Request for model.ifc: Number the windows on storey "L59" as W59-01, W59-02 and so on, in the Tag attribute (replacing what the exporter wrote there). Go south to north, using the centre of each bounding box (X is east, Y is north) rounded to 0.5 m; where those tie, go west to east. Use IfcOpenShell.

First a look at what the model holds.

```python
import ifcopenshell
import ifcopenshell.util.element
import ifcopenshell.util.placement

model = ifcopenshell.open("model.ifc")
print(model.schema)
storey = next(s for s in model.by_type("IfcBuildingStorey") if s.Name == "L59")
windows = [e for e in ifcopenshell.util.element.get_decomposition(storey) if e.is_a("IfcWindow")]
for e in sorted(windows, key=lambda e: e.id()):
    origin = ifcopenshell.util.placement.get_local_placement(e.ObjectPlacement)[:3, 3]
    print(e.id(), e.Tag, e.Name, origin.round(2) + 0.0, sep=" | ")
```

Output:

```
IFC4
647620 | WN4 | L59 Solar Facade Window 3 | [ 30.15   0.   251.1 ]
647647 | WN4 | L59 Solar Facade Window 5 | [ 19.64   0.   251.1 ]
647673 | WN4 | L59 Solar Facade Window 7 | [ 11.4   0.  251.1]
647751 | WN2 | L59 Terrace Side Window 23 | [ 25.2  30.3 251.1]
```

```python
import ifcopenshell
import ifcopenshell.geom
import ifcopenshell.util.element
import ifcopenshell.util.shape

model = ifcopenshell.open("model.ifc")
settings = ifcopenshell.geom.settings()
settings.set("use-world-coords", True)


def centre(element):
    shape = ifcopenshell.geom.create_shape(settings, element)
    return ifcopenshell.util.shape.get_bbox_centroid(shape.geometry)


storey = next(s for s in model.by_type("IfcBuildingStorey") if s.Name == "L59")
windows = [e for e in ifcopenshell.util.element.get_decomposition(storey) if e.is_a("IfcWindow")]

# Insertion points can sit at a corner or the storey origin, so sort by the geometry (in metres).
centres = {e: centre(e) for e in windows}
windows.sort(key=lambda e: (round(centres[e][1] / 0.5), centres[e][0]))

for i, e in enumerate(windows, start=1):
    number = f"W59-{i:02d}"
    e.Tag = number
    print(e.id(), number)

model.write("model_edited.ifc")
```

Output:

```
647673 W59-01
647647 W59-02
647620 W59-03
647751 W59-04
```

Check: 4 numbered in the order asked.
